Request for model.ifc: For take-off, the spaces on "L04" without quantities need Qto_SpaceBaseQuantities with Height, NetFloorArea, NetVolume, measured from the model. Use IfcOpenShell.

First a look at what the model holds.

```python
import ifcopenshell
import ifcopenshell.util.element
import ifcopenshell.util.unit

model = ifcopenshell.open("model.ifc")
print(model.schema)
for unit_type in ("LENGTHUNIT", "AREAUNIT", "VOLUMEUNIT"):
    print(unit_type, ifcopenshell.util.unit.calculate_unit_scale(model, unit_type))
storey = next(s for s in model.by_type("IfcBuildingStorey") if s.Name == "L04")
spaces = [e for e in ifcopenshell.util.element.get_decomposition(storey) if e.is_a("IfcSpace")]
for e in sorted(spaces, key=lambda e: e.id()):
    print(e.id(), e.is_a(), e.Name, list(ifcopenshell.util.element.get_psets(e, qtos_only=True)), sep=" | ")
```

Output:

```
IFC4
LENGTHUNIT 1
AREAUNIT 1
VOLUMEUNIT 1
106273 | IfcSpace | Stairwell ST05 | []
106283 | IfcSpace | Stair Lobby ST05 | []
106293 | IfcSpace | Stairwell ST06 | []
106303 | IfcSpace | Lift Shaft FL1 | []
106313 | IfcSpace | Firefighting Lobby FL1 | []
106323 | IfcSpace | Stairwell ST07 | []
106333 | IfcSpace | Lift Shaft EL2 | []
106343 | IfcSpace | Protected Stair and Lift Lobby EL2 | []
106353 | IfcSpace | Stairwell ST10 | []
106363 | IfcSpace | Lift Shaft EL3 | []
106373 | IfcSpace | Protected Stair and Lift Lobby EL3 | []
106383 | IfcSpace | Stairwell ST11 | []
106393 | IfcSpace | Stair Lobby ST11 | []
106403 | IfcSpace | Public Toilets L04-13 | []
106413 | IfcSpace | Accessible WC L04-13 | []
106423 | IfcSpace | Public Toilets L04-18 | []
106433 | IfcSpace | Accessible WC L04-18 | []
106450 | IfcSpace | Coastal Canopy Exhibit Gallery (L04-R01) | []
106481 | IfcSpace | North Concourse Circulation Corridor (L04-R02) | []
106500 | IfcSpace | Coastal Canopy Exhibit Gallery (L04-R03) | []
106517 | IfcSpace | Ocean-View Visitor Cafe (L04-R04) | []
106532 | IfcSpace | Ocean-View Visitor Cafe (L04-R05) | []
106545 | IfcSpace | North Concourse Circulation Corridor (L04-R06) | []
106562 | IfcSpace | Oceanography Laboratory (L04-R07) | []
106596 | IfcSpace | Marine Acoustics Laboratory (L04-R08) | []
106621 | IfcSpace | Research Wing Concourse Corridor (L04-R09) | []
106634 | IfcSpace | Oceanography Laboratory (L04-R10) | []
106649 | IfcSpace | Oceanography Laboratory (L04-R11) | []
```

```python
import ifcopenshell
import ifcopenshell.api.pset
import ifcopenshell.geom
import ifcopenshell.util.element
import ifcopenshell.util.shape
import ifcopenshell.util.unit

model = ifcopenshell.open("model.ifc")
unit_scale = ifcopenshell.util.unit.calculate_unit_scale(model)
area_scale = ifcopenshell.util.unit.calculate_unit_scale(model, "AREAUNIT")
volume_scale = ifcopenshell.util.unit.calculate_unit_scale(model, "VOLUMEUNIT")
settings = ifcopenshell.geom.settings()

storey = next(s for s in model.by_type("IfcBuildingStorey") if s.Name == "L04")
spaces = [e for e in ifcopenshell.util.element.get_decomposition(storey) if e.is_a("IfcSpace")]

for e in sorted(spaces, key=lambda e: e.id()):
    if ifcopenshell.util.element.get_psets(e, qtos_only=True, should_inherit=False):
        continue
    # Geometry comes back in metres, in the element's own axes.
    shape = ifcopenshell.geom.create_shape(settings, e)
    values = {
        "Height": ifcopenshell.util.shape.get_z(shape.geometry) / unit_scale,
        "NetFloorArea": ifcopenshell.util.shape.get_footprint_area(shape.geometry) / area_scale,
        "NetVolume": ifcopenshell.util.shape.get_volume(shape.geometry) / volume_scale,
    }
    qto = ifcopenshell.api.pset.add_qto(model, product=e, name="Qto_SpaceBaseQuantities")
    ifcopenshell.api.pset.edit_qto(model, qto=qto, properties=values)
    print(e.id(), {k: round(v, 3) for k, v in values.items()})

model.write("model_edited.ifc")
```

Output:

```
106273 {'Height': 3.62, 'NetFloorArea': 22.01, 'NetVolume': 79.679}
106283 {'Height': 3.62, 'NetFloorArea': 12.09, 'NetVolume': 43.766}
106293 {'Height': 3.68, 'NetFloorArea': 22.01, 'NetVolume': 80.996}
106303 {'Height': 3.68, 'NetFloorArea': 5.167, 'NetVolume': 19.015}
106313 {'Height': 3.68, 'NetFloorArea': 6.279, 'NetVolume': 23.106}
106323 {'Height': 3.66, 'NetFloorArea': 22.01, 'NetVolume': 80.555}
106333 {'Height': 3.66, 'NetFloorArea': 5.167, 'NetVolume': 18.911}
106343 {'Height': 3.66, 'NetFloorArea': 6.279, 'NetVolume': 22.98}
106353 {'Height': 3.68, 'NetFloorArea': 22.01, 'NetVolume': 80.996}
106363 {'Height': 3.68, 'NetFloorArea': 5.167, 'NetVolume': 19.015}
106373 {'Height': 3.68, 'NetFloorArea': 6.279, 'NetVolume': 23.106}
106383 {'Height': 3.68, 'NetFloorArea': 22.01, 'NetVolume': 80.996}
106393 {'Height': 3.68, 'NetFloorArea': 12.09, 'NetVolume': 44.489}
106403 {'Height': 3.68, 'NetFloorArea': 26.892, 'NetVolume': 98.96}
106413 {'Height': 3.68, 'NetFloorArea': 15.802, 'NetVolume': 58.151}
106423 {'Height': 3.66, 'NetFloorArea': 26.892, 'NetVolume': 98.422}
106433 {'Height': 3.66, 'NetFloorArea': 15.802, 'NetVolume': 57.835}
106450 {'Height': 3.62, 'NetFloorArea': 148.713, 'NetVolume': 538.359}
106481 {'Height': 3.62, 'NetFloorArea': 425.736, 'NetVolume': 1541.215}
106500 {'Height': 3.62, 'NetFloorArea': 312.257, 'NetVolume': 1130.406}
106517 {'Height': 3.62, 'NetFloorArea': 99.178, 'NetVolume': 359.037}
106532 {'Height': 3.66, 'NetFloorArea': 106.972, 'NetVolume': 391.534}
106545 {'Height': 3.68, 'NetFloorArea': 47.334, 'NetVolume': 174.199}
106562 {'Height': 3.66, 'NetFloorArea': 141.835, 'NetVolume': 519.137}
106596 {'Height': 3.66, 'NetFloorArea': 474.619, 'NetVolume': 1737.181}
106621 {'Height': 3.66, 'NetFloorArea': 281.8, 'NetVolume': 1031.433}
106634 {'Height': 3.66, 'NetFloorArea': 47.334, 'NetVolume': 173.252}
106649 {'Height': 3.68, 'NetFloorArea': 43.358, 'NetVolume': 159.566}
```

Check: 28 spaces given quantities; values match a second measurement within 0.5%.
